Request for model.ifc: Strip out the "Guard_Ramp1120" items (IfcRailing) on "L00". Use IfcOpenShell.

First a look at what the model holds.

```python
import ifcopenshell
import ifcopenshell.util.element

model = ifcopenshell.open("model.ifc")
print(model.schema)
storey = next(s for s in model.by_type("IfcBuildingStorey") if s.Name == "L00")
railings = [e for e in ifcopenshell.util.element.get_decomposition(storey) if e.is_a("IfcRailing")]
seen = {}
for e in railings:
    element_type = ifcopenshell.util.element.get_type(e)
    name = element_type.Name if element_type not in (None, e) else None
    seen[name] = seen.get(name, 0) + 1
for name, count in sorted(seen.items(), key=str):
    print(count, "x", name)
```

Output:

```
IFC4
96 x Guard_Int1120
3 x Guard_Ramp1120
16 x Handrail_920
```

```python
import ifcopenshell
import ifcopenshell.api.root
import ifcopenshell.util.element

model = ifcopenshell.open("model.ifc")

storey = next(s for s in model.by_type("IfcBuildingStorey") if s.Name == "L00")
railings = [e for e in ifcopenshell.util.element.get_decomposition(storey) if e.is_a("IfcRailing")]
targets = [e for e in railings if (t := ifcopenshell.util.element.get_type(e)) not in (None, e) and t.Name == "Guard_Ramp1120"]

for e in targets:
    ifcopenshell.api.root.remove_product(model, product=e)
print(len(targets), "removed")

model.write("model_edited.ifc")
```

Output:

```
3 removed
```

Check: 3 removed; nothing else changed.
